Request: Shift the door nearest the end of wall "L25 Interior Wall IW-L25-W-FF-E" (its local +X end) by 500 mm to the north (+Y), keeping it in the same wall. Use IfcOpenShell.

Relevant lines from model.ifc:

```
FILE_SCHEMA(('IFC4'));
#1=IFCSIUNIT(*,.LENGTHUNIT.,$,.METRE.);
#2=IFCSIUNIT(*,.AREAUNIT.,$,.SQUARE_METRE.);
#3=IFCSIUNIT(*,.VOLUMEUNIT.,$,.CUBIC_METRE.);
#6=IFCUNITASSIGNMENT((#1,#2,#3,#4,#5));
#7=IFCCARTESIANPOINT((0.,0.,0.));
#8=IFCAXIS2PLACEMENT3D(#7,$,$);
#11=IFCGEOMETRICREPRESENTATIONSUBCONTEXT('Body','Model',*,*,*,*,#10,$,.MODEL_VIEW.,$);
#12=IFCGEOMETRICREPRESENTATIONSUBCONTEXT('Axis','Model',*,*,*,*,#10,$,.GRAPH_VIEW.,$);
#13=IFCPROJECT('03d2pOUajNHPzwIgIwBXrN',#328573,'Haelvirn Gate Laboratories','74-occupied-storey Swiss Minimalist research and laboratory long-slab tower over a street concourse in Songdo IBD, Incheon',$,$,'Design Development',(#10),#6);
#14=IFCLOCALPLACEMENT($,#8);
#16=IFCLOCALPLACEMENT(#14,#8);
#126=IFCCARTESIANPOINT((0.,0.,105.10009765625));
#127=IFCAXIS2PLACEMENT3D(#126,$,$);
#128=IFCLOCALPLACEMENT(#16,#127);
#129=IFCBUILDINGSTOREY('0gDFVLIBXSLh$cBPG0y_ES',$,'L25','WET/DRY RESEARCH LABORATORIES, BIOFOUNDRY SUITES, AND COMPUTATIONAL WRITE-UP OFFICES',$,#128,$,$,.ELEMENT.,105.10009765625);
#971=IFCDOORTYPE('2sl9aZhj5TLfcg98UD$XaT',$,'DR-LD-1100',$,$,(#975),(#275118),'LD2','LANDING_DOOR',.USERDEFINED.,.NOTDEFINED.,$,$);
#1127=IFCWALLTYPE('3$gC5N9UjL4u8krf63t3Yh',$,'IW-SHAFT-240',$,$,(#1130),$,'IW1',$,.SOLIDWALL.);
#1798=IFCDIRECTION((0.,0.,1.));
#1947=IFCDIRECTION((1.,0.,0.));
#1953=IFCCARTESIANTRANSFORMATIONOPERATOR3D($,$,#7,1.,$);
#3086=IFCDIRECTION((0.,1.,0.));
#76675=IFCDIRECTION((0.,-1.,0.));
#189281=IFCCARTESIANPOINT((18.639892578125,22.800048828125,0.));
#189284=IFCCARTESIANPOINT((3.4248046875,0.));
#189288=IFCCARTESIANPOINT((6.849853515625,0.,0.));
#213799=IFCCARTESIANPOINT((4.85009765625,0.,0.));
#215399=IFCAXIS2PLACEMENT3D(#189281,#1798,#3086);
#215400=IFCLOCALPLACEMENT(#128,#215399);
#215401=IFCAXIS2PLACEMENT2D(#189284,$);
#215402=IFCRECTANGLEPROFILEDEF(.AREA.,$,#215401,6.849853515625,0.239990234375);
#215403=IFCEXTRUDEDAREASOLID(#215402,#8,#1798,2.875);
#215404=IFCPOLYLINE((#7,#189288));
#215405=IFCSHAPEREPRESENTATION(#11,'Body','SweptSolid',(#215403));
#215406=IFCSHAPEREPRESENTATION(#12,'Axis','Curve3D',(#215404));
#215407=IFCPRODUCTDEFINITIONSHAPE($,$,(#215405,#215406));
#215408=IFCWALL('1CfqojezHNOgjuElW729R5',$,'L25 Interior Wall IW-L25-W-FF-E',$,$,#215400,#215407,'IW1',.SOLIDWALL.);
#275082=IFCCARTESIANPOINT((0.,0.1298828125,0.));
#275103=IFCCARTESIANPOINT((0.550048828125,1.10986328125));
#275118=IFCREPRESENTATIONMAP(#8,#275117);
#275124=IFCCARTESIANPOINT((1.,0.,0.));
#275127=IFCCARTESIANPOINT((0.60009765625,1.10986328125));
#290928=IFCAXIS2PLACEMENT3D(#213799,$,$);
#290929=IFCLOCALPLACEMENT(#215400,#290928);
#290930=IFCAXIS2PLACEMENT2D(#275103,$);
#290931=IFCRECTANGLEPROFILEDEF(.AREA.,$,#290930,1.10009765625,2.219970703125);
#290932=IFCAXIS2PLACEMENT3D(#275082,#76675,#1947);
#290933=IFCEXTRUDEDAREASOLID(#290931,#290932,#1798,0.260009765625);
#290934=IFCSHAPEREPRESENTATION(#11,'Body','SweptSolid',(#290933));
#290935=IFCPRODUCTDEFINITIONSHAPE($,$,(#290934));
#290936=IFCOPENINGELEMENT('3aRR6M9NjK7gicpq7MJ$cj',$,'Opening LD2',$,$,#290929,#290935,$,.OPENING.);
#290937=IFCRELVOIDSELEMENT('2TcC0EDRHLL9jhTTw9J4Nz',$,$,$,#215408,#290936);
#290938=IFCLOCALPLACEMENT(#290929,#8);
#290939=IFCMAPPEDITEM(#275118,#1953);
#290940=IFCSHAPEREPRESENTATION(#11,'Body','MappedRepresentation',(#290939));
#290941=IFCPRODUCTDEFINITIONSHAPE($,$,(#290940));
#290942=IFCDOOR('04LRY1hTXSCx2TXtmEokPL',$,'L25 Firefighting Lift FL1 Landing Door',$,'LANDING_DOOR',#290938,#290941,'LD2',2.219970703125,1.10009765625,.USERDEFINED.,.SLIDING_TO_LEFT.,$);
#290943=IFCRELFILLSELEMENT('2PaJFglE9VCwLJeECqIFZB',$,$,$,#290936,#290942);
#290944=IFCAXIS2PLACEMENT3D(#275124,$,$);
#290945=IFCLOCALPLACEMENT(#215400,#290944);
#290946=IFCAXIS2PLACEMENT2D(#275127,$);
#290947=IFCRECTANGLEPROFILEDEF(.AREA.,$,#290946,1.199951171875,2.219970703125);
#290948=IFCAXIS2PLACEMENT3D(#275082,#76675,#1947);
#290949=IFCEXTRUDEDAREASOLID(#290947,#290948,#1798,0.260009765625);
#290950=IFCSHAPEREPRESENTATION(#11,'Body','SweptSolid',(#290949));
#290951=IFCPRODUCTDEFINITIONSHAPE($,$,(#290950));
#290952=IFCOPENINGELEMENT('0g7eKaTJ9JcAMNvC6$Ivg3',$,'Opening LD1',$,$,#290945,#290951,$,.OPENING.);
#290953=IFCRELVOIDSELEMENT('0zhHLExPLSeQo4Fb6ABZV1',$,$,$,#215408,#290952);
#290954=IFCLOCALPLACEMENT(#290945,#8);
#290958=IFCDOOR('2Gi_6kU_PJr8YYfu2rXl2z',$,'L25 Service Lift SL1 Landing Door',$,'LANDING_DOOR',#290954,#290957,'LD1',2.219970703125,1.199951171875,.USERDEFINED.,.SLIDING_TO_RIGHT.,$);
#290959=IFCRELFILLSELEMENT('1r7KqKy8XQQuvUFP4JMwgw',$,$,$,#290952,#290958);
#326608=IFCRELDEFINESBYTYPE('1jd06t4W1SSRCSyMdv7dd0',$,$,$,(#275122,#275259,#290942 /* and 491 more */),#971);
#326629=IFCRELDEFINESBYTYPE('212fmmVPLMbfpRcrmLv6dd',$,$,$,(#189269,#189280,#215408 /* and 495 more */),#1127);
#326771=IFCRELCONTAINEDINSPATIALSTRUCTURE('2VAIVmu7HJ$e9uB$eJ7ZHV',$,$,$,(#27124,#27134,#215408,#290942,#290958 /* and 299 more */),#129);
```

```python
import ifcopenshell
import ifcopenshell.api.geometry
import ifcopenshell.util.placement

model = ifcopenshell.open("model.ifc")

door = model.by_guid("04LRY1hTXSCx2TXtmEokPL")
opening = door.FillsVoids[0].RelatingOpeningElement
wall = opening.VoidsElements[0].RelatingBuildingElement

wall_matrix = ifcopenshell.util.placement.get_local_placement(wall.ObjectPlacement)
shift = wall_matrix[:3, 0] * 0.5
before = ifcopenshell.util.placement.get_local_placement(door.ObjectPlacement)[:3, 3].copy()

# The door is placed relative to its opening, so it follows when the opening moves.
matrix = ifcopenshell.util.placement.get_local_placement(opening.ObjectPlacement)
matrix[:3, 3] += shift
ifcopenshell.api.geometry.edit_object_placement(
    model, product=opening, matrix=matrix, is_si=False, should_transform_children=True
)

after = ifcopenshell.util.placement.get_local_placement(door.ObjectPlacement)[:3, 3]
print("door moved by", (after - before).round(3) + 0.0)

model.write("model_updated.ifc")
```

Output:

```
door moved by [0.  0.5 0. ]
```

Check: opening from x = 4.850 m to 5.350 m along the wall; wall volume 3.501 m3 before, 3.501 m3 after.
